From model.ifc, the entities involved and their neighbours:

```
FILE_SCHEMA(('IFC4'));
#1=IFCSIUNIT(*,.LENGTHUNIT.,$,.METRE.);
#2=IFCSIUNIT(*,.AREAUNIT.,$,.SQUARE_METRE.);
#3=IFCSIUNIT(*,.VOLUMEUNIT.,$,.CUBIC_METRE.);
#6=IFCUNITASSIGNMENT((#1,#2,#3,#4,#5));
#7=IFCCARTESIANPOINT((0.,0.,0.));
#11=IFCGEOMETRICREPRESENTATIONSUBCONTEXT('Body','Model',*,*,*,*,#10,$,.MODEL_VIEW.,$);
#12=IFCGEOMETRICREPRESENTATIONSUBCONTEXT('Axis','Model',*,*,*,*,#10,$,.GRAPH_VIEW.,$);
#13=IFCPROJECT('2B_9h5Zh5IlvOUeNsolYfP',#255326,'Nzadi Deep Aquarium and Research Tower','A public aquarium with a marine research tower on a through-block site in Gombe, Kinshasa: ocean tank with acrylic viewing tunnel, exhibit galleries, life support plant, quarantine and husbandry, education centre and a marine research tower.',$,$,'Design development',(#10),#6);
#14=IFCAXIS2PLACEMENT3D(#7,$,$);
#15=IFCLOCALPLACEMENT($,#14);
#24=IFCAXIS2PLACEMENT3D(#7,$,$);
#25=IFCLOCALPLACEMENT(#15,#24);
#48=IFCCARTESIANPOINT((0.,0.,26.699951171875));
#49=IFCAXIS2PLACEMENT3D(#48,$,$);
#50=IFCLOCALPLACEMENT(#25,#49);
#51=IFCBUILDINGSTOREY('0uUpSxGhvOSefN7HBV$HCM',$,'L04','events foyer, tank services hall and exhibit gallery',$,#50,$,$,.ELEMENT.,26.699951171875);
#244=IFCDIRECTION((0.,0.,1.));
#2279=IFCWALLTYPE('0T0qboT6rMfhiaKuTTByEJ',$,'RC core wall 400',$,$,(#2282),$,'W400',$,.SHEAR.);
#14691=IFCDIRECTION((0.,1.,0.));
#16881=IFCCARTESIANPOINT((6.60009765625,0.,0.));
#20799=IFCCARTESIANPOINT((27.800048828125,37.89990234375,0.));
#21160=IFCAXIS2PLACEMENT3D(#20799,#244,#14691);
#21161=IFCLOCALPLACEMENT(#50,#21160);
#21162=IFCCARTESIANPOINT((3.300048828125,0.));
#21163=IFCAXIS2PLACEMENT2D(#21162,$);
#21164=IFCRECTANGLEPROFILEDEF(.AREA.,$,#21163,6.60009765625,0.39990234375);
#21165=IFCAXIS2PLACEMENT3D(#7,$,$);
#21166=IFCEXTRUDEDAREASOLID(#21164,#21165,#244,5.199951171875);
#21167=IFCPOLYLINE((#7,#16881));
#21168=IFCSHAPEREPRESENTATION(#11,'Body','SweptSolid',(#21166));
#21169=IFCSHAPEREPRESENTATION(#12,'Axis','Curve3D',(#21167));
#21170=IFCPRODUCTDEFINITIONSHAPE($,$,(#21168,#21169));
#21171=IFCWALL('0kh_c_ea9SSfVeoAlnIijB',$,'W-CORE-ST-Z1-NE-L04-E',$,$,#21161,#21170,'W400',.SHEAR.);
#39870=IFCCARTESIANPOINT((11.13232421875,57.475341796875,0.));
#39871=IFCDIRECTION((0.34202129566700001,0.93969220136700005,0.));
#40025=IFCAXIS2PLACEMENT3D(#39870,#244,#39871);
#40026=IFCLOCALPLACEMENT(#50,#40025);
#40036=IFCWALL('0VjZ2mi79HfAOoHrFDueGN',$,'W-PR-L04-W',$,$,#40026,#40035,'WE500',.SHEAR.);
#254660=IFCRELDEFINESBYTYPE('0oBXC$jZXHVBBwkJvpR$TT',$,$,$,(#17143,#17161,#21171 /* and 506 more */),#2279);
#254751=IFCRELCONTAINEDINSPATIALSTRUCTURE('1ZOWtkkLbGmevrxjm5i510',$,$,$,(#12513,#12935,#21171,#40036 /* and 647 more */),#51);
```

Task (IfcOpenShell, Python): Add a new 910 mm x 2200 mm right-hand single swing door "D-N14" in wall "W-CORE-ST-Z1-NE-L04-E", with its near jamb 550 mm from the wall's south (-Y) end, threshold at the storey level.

```python
import numpy as np
import ifcopenshell
import ifcopenshell.api.feature
import ifcopenshell.api.geometry
import ifcopenshell.api.root
import ifcopenshell.api.spatial
import ifcopenshell.geom
import ifcopenshell.util.element
import ifcopenshell.util.placement
import ifcopenshell.util.representation
import ifcopenshell.util.shape
import ifcopenshell.util.unit

model = ifcopenshell.open("model.ifc")
unit_scale = ifcopenshell.util.unit.calculate_unit_scale(model)
settings = ifcopenshell.geom.settings()


def volume(element):
    """Net volume in cubic metres, openings subtracted."""
    shape = ifcopenshell.geom.create_shape(settings, element)
    return ifcopenshell.util.shape.get_volume(shape.geometry)


wall = model.by_id(21171)
storey = ifcopenshell.util.element.get_container(wall, ifc_class="IfcBuildingStorey")
context = ifcopenshell.util.representation.get_context(model, "Model", "Body", "MODEL_VIEW")
before = volume(wall)

width, height, from_end, sill = 0.91, 2.2, 0.55, 0.0  # metres

# The wall runs along its own X axis, and the end named is its -X end.
wall_shape = ifcopenshell.geom.create_shape(settings, wall)
x, y, z = ifcopenshell.util.shape.get_vertices(wall_shape.geometry).T
start = x.min() + from_end
face, thickness = float(y.min()), float(y.max() - y.min())
wall_matrix = ifcopenshell.util.placement.get_local_placement(wall.ObjectPlacement)
level = ifcopenshell.util.placement.get_local_placement(storey.ObjectPlacement)[2, 3]


def in_wall(x, y):
    """Placement at x, y metres in the wall's axes, at sill height."""
    matrix = wall_matrix.copy()
    matrix[:, 3] = wall_matrix @ np.array([x / unit_scale, y / unit_scale, 0.0, 1.0])
    matrix[2, 3] = level + sill / unit_scale
    return matrix


# Opening: a box that overshoots both wall faces by 50 mm.
opening = ifcopenshell.api.root.create_entity(model, ifc_class="IfcOpeningElement", predefined_type="OPENING")
box = ifcopenshell.api.geometry.add_wall_representation(
    model, context=context, length=width, height=height, thickness=thickness + 0.1
)
ifcopenshell.api.geometry.assign_representation(model, product=opening, representation=box)
ifcopenshell.api.geometry.edit_object_placement(model, product=opening, matrix=in_wall(start, face - 0.05), is_si=False)
ifcopenshell.api.feature.add_feature(model, feature=opening, element=wall)

door = ifcopenshell.api.root.create_entity(model, ifc_class="IfcDoor", name="D-N14", predefined_type="DOOR")
door.OverallWidth, door.OverallHeight = width / unit_scale, height / unit_scale
door.OperationType = "SINGLE_SWING_RIGHT"
body = ifcopenshell.api.geometry.add_door_representation(
    model,
    context=context,
    overall_width=door.OverallWidth,
    overall_height=door.OverallHeight,
    operation_type="SINGLE_SWING_RIGHT",
    lining_properties={"LiningDepth": thickness / unit_scale, "ThresholdDepth": thickness / unit_scale},
)
ifcopenshell.api.geometry.assign_representation(model, product=door, representation=body)
ifcopenshell.api.spatial.assign_container(model, products=[door], relating_structure=storey)
ifcopenshell.api.feature.add_filling(model, opening=opening, element=door)

# The lining spans the wall, so the door starts at the wall face.
ifcopenshell.api.geometry.edit_object_placement(model, product=door, matrix=in_wall(start, face), is_si=False)

after = volume(wall)

print(f"wall volume {before:.3f} -> {after:.3f} m3")

model.write("model_edited.ifc")
```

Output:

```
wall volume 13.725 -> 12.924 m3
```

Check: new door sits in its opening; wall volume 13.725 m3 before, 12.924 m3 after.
